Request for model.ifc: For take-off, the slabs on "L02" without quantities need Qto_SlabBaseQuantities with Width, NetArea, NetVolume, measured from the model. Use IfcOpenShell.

First a look at what the model holds.

```python
import ifcopenshell
import ifcopenshell.util.element
import ifcopenshell.util.unit

model = ifcopenshell.open("model.ifc")
print(model.schema)
for unit_type in ("LENGTHUNIT", "AREAUNIT", "VOLUMEUNIT"):
    print(unit_type, ifcopenshell.util.unit.calculate_unit_scale(model, unit_type))
storey = next(s for s in model.by_type("IfcBuildingStorey") if s.Name == "L02")
slabs = [e for e in ifcopenshell.util.element.get_decomposition(storey) if e.is_a("IfcSlab")]
for e in sorted(slabs, key=lambda e: e.id()):
    print(e.id(), e.is_a(), e.Name, list(ifcopenshell.util.element.get_psets(e, qtos_only=True)), sep=" | ")
```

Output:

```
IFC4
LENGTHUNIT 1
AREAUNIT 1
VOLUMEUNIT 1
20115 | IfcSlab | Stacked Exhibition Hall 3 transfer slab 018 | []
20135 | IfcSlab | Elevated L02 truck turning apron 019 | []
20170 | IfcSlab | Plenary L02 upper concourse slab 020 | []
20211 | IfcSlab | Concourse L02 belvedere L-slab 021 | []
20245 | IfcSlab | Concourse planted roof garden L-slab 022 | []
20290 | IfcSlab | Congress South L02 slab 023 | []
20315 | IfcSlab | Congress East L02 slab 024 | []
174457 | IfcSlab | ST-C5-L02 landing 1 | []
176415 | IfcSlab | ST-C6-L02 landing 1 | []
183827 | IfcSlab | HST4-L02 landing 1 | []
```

```python
import ifcopenshell
import ifcopenshell.api.pset
import ifcopenshell.geom
import ifcopenshell.util.element
import ifcopenshell.util.shape
import ifcopenshell.util.unit

model = ifcopenshell.open("model.ifc")
unit_scale = ifcopenshell.util.unit.calculate_unit_scale(model)
area_scale = ifcopenshell.util.unit.calculate_unit_scale(model, "AREAUNIT")
volume_scale = ifcopenshell.util.unit.calculate_unit_scale(model, "VOLUMEUNIT")
settings = ifcopenshell.geom.settings()

storey = next(s for s in model.by_type("IfcBuildingStorey") if s.Name == "L02")
slabs = [e for e in ifcopenshell.util.element.get_decomposition(storey) if e.is_a("IfcSlab")]

for e in sorted(slabs, key=lambda e: e.id()):
    if ifcopenshell.util.element.get_psets(e, qtos_only=True, should_inherit=False):
        continue
    # Geometry comes back in metres, in the element's own axes.
    shape = ifcopenshell.geom.create_shape(settings, e)
    values = {
        "Width": ifcopenshell.util.shape.get_z(shape.geometry) / unit_scale,
        "NetArea": ifcopenshell.util.shape.get_footprint_area(shape.geometry) / area_scale,
        "NetVolume": ifcopenshell.util.shape.get_volume(shape.geometry) / volume_scale,
    }
    qto = ifcopenshell.api.pset.add_qto(model, product=e, name="Qto_SlabBaseQuantities")
    ifcopenshell.api.pset.edit_qto(model, qto=qto, properties=values)
    print(e.id(), {k: round(v, 3) for k, v in values.items()})

model.write("model-out.ifc")
```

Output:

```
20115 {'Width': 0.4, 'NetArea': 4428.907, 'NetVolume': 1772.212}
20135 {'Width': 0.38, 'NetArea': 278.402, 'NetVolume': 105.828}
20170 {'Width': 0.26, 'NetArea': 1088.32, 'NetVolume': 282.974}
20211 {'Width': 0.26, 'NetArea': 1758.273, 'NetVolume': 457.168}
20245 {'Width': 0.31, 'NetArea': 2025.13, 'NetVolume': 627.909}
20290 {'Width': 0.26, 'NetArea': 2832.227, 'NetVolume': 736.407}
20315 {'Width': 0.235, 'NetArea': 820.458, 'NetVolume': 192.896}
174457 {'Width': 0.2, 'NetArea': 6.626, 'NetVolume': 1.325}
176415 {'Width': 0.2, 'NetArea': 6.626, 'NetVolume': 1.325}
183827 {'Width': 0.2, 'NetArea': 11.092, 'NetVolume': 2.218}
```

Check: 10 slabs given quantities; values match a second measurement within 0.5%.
